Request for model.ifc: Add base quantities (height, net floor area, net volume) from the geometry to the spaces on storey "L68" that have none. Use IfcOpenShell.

First a look at what the model holds.

```python
import ifcopenshell
import ifcopenshell.util.element
import ifcopenshell.util.unit

model = ifcopenshell.open("model.ifc")
print(model.schema)
for unit_type in ("LENGTHUNIT", "AREAUNIT", "VOLUMEUNIT"):
    print(unit_type, ifcopenshell.util.unit.calculate_unit_scale(model, unit_type))
storey = next(s for s in model.by_type("IfcBuildingStorey") if s.Name == "L68")
spaces = [e for e in ifcopenshell.util.element.get_decomposition(storey) if e.is_a("IfcSpace")]
for e in sorted(spaces, key=lambda e: e.id()):
    print(e.id(), e.is_a(), e.Name, list(ifcopenshell.util.element.get_psets(e, qtos_only=True)), sep=" | ")
```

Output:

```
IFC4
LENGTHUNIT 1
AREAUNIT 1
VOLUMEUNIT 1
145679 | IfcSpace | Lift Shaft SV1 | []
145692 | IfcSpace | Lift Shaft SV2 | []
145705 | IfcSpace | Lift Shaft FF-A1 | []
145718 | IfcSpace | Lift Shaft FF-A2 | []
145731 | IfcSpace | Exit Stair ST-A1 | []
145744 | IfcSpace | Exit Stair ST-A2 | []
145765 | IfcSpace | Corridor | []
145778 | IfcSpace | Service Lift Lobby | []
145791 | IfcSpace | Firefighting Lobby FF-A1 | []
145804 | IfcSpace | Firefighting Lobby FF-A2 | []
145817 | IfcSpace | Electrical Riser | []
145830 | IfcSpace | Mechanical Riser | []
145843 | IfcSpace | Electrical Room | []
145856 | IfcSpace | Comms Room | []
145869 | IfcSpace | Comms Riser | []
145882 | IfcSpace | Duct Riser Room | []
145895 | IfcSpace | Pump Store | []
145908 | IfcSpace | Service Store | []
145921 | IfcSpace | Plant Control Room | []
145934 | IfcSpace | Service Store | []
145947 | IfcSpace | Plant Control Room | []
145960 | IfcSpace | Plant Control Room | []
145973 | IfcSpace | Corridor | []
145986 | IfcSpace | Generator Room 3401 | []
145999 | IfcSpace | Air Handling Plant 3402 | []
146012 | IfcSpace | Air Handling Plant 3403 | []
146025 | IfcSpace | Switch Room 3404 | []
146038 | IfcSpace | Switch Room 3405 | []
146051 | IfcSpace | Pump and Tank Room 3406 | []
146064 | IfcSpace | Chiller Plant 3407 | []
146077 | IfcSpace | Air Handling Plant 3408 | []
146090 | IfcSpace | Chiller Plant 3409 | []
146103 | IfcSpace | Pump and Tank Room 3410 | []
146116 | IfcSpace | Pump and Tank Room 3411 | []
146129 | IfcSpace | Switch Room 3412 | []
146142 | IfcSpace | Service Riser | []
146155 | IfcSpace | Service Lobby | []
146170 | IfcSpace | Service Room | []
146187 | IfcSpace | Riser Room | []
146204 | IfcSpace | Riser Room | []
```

```python
import ifcopenshell
import ifcopenshell.api.pset
import ifcopenshell.geom
import ifcopenshell.util.element
import ifcopenshell.util.shape
import ifcopenshell.util.unit

model = ifcopenshell.open("model.ifc")
unit_scale = ifcopenshell.util.unit.calculate_unit_scale(model)
area_scale = ifcopenshell.util.unit.calculate_unit_scale(model, "AREAUNIT")
volume_scale = ifcopenshell.util.unit.calculate_unit_scale(model, "VOLUMEUNIT")
settings = ifcopenshell.geom.settings()

storey = next(s for s in model.by_type("IfcBuildingStorey") if s.Name == "L68")
spaces = [e for e in ifcopenshell.util.element.get_decomposition(storey) if e.is_a("IfcSpace")]

for e in sorted(spaces, key=lambda e: e.id()):
    if ifcopenshell.util.element.get_psets(e, qtos_only=True, should_inherit=False):
        continue
    # Geometry comes back in metres, in the element's own axes.
    shape = ifcopenshell.geom.create_shape(settings, e)
    values = {
        "Height": ifcopenshell.util.shape.get_z(shape.geometry) / unit_scale,
        "NetFloorArea": ifcopenshell.util.shape.get_footprint_area(shape.geometry) / area_scale,
        "NetVolume": ifcopenshell.util.shape.get_volume(shape.geometry) / volume_scale,
    }
    qto = ifcopenshell.api.pset.add_qto(model, product=e, name="Qto_SpaceBaseQuantities")
    ifcopenshell.api.pset.edit_qto(model, qto=qto, properties=values)
    print(e.id(), {k: round(v, 3) for k, v in values.items()})

model.write("model-out.ifc")
```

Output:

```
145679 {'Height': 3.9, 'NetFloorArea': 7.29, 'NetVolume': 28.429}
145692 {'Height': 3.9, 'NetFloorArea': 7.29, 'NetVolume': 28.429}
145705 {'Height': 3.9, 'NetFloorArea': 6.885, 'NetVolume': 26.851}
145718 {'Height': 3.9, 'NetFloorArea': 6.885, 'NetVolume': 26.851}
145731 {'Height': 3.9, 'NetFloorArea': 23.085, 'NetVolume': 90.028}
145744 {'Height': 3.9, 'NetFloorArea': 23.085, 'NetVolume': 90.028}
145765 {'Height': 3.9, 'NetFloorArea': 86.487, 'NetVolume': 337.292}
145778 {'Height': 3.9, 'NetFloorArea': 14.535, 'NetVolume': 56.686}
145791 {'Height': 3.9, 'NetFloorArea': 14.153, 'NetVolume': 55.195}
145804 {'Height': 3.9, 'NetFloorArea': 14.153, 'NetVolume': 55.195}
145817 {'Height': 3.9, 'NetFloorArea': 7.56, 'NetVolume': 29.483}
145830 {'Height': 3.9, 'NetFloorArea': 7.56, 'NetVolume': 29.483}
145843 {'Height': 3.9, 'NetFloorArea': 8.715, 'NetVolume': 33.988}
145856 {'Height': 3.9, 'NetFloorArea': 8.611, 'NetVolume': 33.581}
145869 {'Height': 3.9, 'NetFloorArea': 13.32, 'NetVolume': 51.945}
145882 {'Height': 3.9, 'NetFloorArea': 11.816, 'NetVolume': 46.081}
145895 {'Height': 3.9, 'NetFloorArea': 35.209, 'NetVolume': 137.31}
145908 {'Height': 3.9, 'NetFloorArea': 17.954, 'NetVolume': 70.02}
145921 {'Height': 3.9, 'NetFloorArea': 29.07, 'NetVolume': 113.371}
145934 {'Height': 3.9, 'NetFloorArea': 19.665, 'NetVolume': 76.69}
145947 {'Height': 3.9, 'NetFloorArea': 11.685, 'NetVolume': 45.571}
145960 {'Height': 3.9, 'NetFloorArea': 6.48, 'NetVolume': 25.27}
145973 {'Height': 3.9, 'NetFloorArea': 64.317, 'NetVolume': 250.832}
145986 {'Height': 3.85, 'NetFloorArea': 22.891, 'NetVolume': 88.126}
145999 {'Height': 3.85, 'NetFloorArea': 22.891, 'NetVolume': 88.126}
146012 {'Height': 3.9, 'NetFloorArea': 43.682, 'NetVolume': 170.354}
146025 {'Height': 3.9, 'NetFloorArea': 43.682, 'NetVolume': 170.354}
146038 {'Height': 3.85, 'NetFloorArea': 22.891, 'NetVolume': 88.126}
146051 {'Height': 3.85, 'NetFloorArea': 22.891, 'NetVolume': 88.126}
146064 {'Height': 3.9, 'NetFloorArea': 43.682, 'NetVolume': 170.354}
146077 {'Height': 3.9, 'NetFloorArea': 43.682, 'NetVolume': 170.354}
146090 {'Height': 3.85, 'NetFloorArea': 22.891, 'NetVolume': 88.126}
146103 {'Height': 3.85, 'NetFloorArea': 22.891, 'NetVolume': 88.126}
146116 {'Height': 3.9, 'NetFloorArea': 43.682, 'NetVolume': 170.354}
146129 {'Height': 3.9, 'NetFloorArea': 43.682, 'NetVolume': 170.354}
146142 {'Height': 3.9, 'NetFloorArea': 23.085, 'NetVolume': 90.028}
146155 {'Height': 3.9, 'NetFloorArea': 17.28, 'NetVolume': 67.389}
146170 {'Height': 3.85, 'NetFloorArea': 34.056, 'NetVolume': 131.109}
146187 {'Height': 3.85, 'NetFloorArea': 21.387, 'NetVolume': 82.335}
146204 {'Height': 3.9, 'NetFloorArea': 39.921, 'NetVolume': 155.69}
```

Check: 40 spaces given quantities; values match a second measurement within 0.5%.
